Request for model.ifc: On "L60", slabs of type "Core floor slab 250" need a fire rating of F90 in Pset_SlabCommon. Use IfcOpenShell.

First a look at what the model holds.

```python
import ifcopenshell
import ifcopenshell.util.element

model = ifcopenshell.open("model.ifc")
print(model.schema)
storey = next(s for s in model.by_type("IfcBuildingStorey") if s.Name == "L60")
slabs = [e for e in ifcopenshell.util.element.get_decomposition(storey) if e.is_a("IfcSlab")]
seen = {}
for e in slabs:
    element_type = ifcopenshell.util.element.get_type(e)
    key = (element_type.Name if element_type != e and element_type else None, ifcopenshell.util.element.get_pset(e, "Pset_SlabCommon", "FireRating"))
    seen[key] = seen.get(key, 0) + 1
for (name, value), count in sorted(seen.items(), key=str):
    print(count, "x", name, "|", value)
```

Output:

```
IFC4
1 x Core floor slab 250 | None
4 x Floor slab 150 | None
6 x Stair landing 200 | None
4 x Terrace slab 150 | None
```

```python
import ifcopenshell
import ifcopenshell.api.pset
import ifcopenshell.util.element

model = ifcopenshell.open("model.ifc")

storey = next(s for s in model.by_type("IfcBuildingStorey") if s.Name == "L60")
slabs = [e for e in ifcopenshell.util.element.get_decomposition(storey) if e.is_a("IfcSlab")]

count = 0
for e in slabs:
    element_type = ifcopenshell.util.element.get_type(e)
    if element_type in (None, e) or element_type.Name != "Core floor slab 250":
        continue
    # add_pset returns the element's existing set when there is one.
    pset = ifcopenshell.api.pset.add_pset(model, product=e, name="Pset_SlabCommon")
    ifcopenshell.api.pset.edit_pset(model, pset=pset, properties={"FireRating": "F90"})
    count += 1

print(count, "slabs updated")

model.write("model_v2.ifc")
```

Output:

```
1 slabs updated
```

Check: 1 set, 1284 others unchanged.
